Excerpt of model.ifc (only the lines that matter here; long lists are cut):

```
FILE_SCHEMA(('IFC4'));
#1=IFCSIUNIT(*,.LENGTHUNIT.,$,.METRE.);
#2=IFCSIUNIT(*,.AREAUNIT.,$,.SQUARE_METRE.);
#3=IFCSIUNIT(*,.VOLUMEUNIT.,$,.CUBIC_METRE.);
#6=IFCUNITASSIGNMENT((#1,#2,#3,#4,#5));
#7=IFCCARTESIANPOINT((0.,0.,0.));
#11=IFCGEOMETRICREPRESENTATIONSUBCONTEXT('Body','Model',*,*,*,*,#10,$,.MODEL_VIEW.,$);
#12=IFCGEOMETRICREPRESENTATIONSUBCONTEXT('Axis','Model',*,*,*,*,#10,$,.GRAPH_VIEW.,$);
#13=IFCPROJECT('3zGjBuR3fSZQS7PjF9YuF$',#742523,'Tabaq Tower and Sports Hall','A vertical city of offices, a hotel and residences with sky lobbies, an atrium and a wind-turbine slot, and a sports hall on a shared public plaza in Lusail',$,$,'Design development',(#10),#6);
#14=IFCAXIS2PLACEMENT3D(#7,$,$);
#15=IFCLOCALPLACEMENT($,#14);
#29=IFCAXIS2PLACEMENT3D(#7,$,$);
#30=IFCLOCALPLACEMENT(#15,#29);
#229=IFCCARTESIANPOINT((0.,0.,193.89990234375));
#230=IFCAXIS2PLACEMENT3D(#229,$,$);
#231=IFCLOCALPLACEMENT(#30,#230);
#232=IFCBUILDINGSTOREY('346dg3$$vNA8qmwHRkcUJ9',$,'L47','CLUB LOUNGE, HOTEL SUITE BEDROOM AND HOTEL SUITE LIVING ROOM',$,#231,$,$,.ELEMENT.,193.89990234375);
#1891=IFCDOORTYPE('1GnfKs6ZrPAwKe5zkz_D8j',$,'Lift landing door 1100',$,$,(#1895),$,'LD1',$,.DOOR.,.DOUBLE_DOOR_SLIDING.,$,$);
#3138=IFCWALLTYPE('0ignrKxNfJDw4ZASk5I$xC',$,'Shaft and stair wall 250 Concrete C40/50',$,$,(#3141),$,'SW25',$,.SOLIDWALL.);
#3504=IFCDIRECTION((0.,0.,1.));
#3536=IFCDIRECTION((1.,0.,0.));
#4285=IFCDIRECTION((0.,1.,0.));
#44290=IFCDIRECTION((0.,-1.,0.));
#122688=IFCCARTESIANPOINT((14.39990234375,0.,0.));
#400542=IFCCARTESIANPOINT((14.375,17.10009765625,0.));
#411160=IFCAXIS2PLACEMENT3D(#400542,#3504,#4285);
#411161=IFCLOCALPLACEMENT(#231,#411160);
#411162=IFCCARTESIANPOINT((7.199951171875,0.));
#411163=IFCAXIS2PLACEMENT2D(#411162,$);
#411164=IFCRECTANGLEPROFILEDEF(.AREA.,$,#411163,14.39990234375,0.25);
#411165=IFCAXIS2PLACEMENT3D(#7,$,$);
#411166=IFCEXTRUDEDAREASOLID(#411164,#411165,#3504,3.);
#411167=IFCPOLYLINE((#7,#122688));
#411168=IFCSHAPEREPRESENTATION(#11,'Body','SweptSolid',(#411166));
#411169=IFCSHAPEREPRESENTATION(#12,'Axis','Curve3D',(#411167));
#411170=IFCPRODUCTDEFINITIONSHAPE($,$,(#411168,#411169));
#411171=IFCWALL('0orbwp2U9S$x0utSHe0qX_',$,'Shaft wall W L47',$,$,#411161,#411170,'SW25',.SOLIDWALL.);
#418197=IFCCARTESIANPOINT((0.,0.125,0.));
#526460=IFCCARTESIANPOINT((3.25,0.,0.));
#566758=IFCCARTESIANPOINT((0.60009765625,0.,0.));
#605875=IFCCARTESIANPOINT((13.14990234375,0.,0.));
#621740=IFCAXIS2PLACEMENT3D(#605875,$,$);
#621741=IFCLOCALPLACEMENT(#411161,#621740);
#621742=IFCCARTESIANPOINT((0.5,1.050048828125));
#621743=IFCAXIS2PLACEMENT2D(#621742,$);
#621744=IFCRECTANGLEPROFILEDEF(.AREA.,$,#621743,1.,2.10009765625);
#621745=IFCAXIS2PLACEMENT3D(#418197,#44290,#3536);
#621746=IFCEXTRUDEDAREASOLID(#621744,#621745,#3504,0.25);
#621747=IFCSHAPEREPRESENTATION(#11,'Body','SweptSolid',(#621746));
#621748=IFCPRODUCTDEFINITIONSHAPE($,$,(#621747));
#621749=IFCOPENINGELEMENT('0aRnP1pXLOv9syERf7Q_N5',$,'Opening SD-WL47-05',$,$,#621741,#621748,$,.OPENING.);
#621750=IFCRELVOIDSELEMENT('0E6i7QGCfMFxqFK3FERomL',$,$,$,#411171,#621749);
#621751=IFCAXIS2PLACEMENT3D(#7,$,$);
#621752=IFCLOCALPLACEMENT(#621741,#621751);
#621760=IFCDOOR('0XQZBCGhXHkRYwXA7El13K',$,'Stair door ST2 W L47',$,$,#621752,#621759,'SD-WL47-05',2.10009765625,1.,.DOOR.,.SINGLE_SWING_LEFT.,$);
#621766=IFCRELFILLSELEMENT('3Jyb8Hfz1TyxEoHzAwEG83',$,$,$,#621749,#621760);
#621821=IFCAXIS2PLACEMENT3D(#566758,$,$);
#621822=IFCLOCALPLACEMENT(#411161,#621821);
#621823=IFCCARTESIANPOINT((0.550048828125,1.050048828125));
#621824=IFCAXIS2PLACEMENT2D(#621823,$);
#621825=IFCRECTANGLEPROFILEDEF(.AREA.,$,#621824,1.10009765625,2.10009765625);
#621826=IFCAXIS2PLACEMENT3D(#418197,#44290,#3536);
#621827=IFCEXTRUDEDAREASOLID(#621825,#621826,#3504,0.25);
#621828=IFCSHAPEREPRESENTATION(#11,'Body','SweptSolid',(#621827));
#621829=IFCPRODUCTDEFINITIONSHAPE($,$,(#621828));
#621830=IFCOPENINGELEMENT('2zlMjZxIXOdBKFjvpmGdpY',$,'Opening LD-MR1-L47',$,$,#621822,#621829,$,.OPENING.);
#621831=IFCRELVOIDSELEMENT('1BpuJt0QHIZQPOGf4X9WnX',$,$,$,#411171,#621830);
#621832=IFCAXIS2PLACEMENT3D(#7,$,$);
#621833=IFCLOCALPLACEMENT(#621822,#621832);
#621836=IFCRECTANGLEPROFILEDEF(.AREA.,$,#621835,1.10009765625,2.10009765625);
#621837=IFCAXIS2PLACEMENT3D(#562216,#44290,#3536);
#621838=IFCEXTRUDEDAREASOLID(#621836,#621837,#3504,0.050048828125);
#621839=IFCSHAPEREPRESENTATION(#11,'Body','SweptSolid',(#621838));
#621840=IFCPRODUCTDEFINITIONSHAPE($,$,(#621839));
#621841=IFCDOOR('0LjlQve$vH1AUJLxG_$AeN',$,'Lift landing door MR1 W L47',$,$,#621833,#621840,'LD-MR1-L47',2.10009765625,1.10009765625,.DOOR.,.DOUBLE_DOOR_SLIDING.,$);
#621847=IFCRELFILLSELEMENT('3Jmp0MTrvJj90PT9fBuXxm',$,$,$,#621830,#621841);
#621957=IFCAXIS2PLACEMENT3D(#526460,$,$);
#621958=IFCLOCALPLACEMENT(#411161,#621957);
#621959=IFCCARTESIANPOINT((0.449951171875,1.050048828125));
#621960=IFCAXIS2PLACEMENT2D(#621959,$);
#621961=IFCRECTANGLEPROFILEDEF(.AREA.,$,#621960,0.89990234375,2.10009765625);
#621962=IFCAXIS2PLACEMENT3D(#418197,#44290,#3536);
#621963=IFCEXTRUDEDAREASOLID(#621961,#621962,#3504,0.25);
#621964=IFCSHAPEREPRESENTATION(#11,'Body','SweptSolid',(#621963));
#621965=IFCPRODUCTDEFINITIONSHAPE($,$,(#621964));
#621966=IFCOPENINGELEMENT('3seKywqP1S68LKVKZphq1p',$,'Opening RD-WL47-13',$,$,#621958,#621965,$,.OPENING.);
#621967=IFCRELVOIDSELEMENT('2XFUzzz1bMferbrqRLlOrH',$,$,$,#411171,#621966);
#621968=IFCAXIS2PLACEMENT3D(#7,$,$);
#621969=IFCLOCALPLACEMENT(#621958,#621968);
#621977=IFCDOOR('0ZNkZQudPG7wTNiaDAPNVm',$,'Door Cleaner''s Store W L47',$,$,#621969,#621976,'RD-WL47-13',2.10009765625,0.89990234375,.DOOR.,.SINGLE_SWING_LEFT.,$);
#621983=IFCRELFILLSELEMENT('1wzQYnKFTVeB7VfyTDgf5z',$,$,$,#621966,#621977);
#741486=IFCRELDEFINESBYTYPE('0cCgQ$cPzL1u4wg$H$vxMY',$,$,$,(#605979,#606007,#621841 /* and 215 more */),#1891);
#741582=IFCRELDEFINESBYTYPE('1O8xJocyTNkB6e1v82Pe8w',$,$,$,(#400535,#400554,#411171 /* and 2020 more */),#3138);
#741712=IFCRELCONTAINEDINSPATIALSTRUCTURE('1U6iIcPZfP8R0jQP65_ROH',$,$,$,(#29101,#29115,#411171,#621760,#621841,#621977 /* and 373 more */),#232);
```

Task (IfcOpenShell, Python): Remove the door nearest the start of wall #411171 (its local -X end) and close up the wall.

```python
import ifcopenshell
import ifcopenshell.api.feature
import ifcopenshell.api.root
import ifcopenshell.geom
import ifcopenshell.util.shape

model = ifcopenshell.open("model.ifc")
settings = ifcopenshell.geom.settings()


def volume(element):
    """Net volume in cubic metres, openings subtracted."""
    shape = ifcopenshell.geom.create_shape(settings, element)
    return ifcopenshell.util.shape.get_volume(shape.geometry)


door = model.by_id(621841)
opening = door.FillsVoids[0].RelatingOpeningElement
wall = opening.VoidsElements[0].RelatingBuildingElement
before = volume(wall)

ifcopenshell.api.root.remove_product(model, product=door)
ifcopenshell.api.feature.remove_feature(model, feature=opening)

after = volume(wall)

print(f"wall volume {before:.3f} -> {after:.3f} m3")

model.write("model_edited.ifc")
```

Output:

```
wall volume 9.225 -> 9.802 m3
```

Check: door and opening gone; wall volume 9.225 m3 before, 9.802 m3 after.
